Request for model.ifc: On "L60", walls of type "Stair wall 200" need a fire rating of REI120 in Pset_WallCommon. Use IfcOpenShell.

First a look at what the model holds.

```python
import ifcopenshell
import ifcopenshell.util.element

model = ifcopenshell.open("model.ifc")
print(model.schema)
storey = next(s for s in model.by_type("IfcBuildingStorey") if s.Name == "L60")
walls = [e for e in ifcopenshell.util.element.get_decomposition(storey) if e.is_a("IfcWall")]
seen = {}
for e in walls:
    element_type = ifcopenshell.util.element.get_type(e)
    key = (element_type.Name if element_type != e and element_type else None, ifcopenshell.util.element.get_pset(e, "Pset_WallCommon", "FireRating"))
    seen[key] = seen.get(key, 0) + 1
for (name, value), count in sorted(seen.items(), key=str):
    print(count, "x", name, "|", value)
```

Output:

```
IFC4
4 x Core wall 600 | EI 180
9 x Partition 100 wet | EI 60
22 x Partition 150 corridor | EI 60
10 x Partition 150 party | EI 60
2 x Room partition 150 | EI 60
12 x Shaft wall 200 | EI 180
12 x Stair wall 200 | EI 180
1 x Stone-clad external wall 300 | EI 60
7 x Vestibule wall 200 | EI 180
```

```python
import ifcopenshell
import ifcopenshell.api.pset
import ifcopenshell.util.element

model = ifcopenshell.open("model.ifc")

storey = next(s for s in model.by_type("IfcBuildingStorey") if s.Name == "L60")
walls = [e for e in ifcopenshell.util.element.get_decomposition(storey) if e.is_a("IfcWall")]

count = 0
for e in walls:
    element_type = ifcopenshell.util.element.get_type(e)
    if element_type in (None, e) or element_type.Name != "Stair wall 200":
        continue
    found = ifcopenshell.util.element.get_pset(e, "Pset_WallCommon", should_inherit=False)
    if found:
        pset = model.by_id(found["id"])
        if len(ifcopenshell.util.element.get_elements_by_pset(pset)) > 1:
            pset = ifcopenshell.api.pset.unshare_pset(model, products=[e], pset=pset)[0]
    else:
        pset = ifcopenshell.api.pset.add_pset(model, product=e, name="Pset_WallCommon")
    ifcopenshell.api.pset.edit_pset(model, pset=pset, properties={"FireRating": "REI120"})
    count += 1

print(count, "walls updated")

model.write("model_updated.ifc")
```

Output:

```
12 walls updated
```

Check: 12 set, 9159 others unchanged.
